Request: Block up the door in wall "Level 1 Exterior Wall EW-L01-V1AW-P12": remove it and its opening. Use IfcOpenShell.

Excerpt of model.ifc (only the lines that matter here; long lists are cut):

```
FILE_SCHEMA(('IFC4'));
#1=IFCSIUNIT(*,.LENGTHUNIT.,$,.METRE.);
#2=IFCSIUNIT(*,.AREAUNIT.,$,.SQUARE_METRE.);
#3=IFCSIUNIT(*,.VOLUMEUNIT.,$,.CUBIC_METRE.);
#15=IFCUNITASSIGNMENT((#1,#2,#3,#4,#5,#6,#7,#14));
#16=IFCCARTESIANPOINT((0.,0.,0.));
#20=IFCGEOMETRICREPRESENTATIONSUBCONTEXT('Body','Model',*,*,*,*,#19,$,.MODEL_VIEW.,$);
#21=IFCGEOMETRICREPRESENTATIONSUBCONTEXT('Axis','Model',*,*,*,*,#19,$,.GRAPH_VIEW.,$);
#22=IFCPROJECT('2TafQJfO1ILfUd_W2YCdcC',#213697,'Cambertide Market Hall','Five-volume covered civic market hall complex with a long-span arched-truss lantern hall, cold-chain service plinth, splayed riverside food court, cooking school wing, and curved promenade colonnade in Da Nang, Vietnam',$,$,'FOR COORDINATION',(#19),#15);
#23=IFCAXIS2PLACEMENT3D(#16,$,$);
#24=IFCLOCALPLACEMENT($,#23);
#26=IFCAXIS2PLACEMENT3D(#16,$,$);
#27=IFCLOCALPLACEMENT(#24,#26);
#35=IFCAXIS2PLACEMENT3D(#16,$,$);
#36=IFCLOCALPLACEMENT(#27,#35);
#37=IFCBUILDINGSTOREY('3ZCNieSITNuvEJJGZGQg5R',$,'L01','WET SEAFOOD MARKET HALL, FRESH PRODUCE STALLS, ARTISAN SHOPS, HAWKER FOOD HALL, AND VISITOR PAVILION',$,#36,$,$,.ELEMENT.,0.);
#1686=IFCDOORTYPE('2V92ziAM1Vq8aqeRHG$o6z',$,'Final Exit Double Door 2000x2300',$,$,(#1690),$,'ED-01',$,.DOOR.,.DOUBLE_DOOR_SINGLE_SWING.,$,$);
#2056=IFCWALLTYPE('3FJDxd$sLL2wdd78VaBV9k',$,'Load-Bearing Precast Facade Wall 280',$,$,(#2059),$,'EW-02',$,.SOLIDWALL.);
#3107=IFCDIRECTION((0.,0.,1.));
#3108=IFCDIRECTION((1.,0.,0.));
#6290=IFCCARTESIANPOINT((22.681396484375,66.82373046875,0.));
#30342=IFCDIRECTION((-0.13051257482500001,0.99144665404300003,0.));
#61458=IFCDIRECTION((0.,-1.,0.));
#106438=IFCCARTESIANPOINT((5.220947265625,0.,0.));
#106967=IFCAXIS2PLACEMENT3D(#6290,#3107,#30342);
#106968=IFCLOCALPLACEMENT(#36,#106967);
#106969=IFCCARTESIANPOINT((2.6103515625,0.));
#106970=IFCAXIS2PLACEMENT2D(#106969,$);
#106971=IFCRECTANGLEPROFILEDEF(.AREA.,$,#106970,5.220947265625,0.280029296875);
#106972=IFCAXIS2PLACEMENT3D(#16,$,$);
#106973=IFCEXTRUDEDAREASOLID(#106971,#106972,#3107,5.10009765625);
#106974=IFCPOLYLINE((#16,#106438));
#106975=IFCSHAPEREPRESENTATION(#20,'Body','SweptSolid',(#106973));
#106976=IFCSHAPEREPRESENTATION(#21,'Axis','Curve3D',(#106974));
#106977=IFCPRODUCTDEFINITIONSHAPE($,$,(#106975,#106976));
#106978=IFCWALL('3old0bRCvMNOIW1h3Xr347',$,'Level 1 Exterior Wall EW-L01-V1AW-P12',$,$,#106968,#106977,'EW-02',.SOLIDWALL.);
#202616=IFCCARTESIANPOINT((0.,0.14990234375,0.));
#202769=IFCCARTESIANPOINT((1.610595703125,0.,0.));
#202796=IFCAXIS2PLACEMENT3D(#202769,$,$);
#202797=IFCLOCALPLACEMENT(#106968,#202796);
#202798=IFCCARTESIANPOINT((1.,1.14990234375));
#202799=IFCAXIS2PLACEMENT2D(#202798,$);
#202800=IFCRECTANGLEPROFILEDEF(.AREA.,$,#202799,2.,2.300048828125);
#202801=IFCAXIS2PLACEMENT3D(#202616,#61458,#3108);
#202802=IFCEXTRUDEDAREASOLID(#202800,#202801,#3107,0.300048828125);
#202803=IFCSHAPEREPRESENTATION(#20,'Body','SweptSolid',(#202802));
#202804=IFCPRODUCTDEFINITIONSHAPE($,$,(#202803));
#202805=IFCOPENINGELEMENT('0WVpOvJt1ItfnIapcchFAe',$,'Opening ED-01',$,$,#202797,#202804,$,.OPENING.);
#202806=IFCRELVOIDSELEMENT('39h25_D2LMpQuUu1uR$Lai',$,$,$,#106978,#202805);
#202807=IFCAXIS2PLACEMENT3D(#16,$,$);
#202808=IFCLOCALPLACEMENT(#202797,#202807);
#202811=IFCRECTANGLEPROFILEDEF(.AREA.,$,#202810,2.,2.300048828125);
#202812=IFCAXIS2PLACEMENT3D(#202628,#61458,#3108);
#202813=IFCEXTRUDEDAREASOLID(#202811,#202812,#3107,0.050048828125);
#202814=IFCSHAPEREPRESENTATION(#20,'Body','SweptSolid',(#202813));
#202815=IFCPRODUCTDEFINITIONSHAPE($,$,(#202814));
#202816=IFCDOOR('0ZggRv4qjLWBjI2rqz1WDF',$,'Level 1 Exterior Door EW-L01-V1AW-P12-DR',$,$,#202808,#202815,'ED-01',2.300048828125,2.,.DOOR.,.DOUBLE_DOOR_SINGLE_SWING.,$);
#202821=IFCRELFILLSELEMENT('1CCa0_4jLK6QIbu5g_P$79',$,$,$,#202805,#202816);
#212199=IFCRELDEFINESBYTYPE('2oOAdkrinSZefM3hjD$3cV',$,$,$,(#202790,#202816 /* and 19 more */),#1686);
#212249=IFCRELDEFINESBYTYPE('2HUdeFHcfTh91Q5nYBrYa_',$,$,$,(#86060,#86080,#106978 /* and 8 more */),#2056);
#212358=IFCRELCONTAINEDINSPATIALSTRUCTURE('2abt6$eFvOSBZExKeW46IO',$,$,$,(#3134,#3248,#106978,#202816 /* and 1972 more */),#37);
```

```python
import ifcopenshell
import ifcopenshell.api.feature
import ifcopenshell.api.root
import ifcopenshell.geom
import ifcopenshell.util.shape

model = ifcopenshell.open("model.ifc")
settings = ifcopenshell.geom.settings()


def volume(element):
    """Net volume in cubic metres, openings subtracted."""
    shape = ifcopenshell.geom.create_shape(settings, element)
    return ifcopenshell.util.shape.get_volume(shape.geometry)


door = model.by_id(202816)
opening = door.FillsVoids[0].RelatingOpeningElement
wall = opening.VoidsElements[0].RelatingBuildingElement
before = volume(wall)

ifcopenshell.api.root.remove_product(model, product=door)
ifcopenshell.api.feature.remove_feature(model, feature=opening)

after = volume(wall)

print(f"wall volume {before:.3f} -> {after:.3f} m3")

model.write("model-out.ifc")
```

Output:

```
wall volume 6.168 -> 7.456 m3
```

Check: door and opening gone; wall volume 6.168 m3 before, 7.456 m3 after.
